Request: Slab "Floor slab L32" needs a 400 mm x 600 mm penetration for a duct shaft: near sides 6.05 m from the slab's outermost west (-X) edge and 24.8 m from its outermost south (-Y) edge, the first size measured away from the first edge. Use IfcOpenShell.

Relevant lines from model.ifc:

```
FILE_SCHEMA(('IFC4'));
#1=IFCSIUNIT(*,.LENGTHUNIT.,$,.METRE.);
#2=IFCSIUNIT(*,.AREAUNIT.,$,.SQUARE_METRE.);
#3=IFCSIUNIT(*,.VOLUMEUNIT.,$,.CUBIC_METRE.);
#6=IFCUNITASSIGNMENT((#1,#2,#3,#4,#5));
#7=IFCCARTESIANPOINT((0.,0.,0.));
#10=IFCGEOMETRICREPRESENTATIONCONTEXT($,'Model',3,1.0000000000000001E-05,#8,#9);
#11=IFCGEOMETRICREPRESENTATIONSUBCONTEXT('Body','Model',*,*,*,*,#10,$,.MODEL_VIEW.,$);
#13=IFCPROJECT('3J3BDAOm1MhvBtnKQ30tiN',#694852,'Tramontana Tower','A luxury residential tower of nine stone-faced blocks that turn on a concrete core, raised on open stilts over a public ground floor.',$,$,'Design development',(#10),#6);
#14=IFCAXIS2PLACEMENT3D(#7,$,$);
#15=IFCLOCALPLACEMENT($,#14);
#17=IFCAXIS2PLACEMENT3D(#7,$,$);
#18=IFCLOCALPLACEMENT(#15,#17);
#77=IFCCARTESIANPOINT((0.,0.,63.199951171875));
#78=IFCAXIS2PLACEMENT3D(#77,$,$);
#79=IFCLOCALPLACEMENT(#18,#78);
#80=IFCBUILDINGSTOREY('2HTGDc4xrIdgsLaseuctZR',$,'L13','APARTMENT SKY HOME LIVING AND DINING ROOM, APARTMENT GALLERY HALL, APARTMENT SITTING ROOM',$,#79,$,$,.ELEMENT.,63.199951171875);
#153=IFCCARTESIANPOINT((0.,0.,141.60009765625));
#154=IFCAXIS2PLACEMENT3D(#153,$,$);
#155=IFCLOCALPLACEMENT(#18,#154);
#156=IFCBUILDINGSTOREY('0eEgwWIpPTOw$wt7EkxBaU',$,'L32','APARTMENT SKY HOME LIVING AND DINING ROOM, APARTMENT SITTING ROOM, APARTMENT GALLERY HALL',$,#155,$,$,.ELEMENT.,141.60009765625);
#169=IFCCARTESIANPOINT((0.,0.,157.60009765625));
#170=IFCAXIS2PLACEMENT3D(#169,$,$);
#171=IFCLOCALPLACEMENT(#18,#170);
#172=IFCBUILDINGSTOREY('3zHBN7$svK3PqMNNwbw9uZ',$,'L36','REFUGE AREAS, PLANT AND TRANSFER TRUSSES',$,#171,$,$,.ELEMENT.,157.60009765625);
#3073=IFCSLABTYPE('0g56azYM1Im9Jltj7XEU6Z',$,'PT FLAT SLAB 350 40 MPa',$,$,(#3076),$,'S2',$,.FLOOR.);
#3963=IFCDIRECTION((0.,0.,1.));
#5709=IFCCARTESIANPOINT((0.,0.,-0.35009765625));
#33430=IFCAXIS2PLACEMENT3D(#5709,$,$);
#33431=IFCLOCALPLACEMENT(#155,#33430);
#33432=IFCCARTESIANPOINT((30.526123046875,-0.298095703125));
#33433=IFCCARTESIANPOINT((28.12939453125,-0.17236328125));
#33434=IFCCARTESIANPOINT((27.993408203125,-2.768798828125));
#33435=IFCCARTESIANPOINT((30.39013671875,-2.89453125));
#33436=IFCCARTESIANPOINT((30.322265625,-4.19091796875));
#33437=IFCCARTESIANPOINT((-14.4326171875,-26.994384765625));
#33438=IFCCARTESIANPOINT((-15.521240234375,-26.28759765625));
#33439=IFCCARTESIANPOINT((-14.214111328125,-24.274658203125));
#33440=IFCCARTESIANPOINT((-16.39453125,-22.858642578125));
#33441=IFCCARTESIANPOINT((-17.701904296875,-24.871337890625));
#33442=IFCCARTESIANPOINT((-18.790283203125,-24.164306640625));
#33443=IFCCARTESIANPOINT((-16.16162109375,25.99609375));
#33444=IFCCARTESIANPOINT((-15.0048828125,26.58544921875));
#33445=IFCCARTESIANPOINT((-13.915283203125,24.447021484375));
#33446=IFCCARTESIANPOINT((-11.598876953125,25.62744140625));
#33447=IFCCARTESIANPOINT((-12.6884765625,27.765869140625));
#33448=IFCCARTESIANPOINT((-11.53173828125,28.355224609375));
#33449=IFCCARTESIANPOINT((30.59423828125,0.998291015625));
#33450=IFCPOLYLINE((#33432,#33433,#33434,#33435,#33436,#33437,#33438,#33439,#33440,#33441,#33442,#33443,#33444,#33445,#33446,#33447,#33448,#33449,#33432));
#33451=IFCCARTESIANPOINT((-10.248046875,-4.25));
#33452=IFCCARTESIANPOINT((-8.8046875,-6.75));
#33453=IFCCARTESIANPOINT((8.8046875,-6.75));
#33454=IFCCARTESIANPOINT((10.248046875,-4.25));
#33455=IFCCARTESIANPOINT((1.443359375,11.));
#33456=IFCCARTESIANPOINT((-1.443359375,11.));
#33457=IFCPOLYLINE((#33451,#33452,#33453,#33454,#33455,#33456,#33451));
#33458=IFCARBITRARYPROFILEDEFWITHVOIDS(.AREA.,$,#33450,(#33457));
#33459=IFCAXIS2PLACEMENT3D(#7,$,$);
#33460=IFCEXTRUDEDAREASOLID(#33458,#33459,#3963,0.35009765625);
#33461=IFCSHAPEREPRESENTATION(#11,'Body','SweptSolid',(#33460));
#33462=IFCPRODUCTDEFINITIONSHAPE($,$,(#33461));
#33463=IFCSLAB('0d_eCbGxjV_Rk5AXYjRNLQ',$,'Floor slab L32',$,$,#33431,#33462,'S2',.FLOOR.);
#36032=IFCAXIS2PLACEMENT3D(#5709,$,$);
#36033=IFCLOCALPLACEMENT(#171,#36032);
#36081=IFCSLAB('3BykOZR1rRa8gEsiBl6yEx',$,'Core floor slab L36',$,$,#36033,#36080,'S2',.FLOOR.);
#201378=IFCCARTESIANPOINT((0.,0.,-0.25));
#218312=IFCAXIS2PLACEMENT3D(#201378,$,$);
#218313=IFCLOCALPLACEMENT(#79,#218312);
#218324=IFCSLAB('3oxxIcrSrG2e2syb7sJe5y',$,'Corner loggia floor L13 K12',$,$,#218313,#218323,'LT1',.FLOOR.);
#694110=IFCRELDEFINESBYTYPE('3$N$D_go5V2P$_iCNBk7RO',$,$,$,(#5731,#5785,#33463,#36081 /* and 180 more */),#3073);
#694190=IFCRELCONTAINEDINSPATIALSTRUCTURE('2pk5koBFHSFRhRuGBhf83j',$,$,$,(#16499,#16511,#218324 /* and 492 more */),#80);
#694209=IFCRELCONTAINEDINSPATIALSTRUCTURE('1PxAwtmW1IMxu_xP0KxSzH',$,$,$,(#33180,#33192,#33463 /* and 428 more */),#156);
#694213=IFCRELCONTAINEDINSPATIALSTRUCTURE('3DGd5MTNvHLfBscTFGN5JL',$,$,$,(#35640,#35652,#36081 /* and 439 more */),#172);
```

```python
import numpy as np
import ifcopenshell
import ifcopenshell.api.feature
import ifcopenshell.api.geometry
import ifcopenshell.api.root
import ifcopenshell.geom
import ifcopenshell.util.placement
import ifcopenshell.util.representation
import ifcopenshell.util.shape
import ifcopenshell.util.unit

model = ifcopenshell.open("model.ifc")
unit_scale = ifcopenshell.util.unit.calculate_unit_scale(model)
settings = ifcopenshell.geom.settings()


def volume(element):
    """Net volume in cubic metres, openings subtracted."""
    shape = ifcopenshell.geom.create_shape(settings, element)
    return ifcopenshell.util.shape.get_volume(shape.geometry)


slab = model.by_id(33463)
before = volume(slab)

# Extent in the slab's own axes, in metres. The edges named are its -X and -Y sides.
slab_shape = ifcopenshell.geom.create_shape(settings, slab)
vertices = ifcopenshell.util.shape.get_vertices(slab_shape.geometry)
x_min, y_min, bottom = vertices.min(axis=0)
top = vertices[:, 2].max()

opening = ifcopenshell.api.root.create_entity(model, ifc_class="IfcOpeningElement", name="Duct shaft opening", predefined_type="OPENING")
context = ifcopenshell.util.representation.get_context(model, "Model", "Body", "MODEL_VIEW")
width, depth = 0.4, 0.6
outline = [(0.0, 0.0), (width, 0.0), (width, depth), (0.0, depth), (0.0, 0.0)]
# Overshoot both faces by 50 mm so the cut is clean.
shape = ifcopenshell.api.geometry.add_slab_representation(
    model, context=context, depth=top - bottom + 0.1, polyline=outline
)
ifcopenshell.api.geometry.assign_representation(model, product=opening, representation=shape)

matrix = ifcopenshell.util.placement.get_local_placement(slab.ObjectPlacement)
matrix[:, 3] = matrix @ np.append(np.array([x_min + 6.05, y_min + 24.8, bottom - 0.05]) / unit_scale, 1.0)
ifcopenshell.api.geometry.edit_object_placement(model, product=opening, matrix=matrix, is_si=False)
ifcopenshell.api.feature.add_feature(model, feature=opening, element=slab)

after = volume(slab)

print(f"slab volume {before:.3f} -> {after:.3f} m3")

model.write("model-out.ifc")
```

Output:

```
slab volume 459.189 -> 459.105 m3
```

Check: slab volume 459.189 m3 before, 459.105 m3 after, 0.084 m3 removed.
